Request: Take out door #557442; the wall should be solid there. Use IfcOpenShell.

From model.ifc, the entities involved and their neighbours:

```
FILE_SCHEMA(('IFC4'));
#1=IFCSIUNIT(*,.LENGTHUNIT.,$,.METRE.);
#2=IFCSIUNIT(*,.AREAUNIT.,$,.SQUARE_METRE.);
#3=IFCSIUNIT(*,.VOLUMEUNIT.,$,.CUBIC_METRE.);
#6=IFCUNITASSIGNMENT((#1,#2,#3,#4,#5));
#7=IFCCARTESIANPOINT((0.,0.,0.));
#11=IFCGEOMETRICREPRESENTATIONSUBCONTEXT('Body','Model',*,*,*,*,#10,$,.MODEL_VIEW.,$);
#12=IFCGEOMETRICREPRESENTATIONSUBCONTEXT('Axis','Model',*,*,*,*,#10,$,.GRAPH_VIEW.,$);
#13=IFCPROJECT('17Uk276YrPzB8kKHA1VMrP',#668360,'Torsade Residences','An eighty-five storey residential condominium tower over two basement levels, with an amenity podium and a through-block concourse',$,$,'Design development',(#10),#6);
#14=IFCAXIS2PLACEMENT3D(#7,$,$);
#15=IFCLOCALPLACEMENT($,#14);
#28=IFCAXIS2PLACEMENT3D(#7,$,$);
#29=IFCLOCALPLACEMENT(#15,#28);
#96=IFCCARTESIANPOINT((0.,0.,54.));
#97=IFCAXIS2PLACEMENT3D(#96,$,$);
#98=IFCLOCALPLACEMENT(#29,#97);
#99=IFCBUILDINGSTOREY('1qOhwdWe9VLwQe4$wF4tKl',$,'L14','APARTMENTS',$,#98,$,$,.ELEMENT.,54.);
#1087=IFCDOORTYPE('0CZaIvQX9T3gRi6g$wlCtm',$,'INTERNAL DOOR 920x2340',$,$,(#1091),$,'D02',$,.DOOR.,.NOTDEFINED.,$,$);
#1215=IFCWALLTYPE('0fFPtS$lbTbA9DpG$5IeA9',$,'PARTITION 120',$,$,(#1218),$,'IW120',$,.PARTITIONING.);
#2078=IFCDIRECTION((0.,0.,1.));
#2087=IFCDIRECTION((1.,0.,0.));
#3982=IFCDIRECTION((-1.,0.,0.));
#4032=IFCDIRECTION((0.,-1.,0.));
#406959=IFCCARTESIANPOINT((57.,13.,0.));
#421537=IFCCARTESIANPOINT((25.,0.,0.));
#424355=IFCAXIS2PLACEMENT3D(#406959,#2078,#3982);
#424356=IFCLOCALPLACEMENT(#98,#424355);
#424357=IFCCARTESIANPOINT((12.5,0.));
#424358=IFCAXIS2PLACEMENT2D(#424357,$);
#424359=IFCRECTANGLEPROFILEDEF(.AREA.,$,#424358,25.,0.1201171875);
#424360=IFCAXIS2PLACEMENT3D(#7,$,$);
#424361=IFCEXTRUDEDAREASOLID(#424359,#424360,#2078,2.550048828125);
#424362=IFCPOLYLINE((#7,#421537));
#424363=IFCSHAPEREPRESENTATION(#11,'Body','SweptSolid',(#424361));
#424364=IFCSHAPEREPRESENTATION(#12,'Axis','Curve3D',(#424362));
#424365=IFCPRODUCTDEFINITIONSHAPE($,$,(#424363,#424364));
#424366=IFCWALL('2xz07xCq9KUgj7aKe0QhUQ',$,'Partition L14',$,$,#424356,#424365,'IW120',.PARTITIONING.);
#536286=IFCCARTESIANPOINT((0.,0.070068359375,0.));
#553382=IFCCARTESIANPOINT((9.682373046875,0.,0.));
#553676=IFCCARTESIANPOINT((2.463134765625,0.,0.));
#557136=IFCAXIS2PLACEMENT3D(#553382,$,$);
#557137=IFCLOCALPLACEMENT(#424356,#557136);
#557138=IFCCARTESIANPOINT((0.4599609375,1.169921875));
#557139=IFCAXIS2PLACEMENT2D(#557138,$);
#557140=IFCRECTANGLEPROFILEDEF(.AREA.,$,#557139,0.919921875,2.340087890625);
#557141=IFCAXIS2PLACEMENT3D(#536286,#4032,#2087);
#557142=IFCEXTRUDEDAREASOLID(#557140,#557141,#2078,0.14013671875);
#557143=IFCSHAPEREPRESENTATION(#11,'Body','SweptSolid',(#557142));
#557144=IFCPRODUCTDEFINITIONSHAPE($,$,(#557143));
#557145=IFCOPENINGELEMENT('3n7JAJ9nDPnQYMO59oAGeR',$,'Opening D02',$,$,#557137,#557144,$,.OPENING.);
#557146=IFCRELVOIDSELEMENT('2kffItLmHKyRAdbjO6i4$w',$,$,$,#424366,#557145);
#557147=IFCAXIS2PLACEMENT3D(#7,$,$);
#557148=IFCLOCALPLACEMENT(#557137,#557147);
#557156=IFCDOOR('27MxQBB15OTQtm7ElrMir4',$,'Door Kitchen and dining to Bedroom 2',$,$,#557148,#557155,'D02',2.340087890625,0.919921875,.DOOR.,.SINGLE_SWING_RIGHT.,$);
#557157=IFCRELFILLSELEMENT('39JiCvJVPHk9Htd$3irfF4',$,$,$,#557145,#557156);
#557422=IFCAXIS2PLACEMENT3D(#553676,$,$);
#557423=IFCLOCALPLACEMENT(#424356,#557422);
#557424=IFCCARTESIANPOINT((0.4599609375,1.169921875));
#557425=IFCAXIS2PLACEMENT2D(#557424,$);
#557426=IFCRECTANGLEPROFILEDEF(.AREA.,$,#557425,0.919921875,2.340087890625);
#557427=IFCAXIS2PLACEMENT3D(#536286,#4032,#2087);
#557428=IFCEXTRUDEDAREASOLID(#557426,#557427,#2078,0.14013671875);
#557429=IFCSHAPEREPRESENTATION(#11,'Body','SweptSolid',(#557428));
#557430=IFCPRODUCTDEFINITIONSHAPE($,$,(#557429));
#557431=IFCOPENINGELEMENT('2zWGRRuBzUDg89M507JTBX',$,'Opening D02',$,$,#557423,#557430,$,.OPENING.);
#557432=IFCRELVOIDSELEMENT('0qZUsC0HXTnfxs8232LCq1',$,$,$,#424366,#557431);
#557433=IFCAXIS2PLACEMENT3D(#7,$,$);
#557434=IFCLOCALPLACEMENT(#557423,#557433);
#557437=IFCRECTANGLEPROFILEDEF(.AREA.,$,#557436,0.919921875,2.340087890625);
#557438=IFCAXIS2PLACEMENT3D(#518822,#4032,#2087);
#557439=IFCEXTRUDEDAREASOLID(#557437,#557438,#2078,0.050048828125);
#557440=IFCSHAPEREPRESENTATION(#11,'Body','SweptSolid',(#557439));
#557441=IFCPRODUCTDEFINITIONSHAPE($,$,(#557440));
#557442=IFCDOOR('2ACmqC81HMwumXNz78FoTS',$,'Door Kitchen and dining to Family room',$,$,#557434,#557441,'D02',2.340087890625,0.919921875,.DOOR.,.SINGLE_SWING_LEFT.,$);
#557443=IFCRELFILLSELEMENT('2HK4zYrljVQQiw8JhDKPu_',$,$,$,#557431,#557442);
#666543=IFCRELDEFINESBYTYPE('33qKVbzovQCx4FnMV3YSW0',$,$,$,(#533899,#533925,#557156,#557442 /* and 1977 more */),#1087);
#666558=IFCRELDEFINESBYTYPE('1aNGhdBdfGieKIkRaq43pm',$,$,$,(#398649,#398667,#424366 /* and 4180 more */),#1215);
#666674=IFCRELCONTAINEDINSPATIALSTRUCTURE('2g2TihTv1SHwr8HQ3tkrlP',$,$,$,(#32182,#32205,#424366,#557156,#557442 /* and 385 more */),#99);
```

```python
import ifcopenshell
import ifcopenshell.api.feature
import ifcopenshell.api.root
import ifcopenshell.geom
import ifcopenshell.util.shape

model = ifcopenshell.open("model.ifc")
settings = ifcopenshell.geom.settings()


def volume(element):
    """Net volume in cubic metres, openings subtracted."""
    shape = ifcopenshell.geom.create_shape(settings, element)
    return ifcopenshell.util.shape.get_volume(shape.geometry)


door = model.by_id(557442)
opening = door.FillsVoids[0].RelatingOpeningElement
wall = opening.VoidsElements[0].RelatingBuildingElement
before = volume(wall)

ifcopenshell.api.root.remove_product(model, product=door)
ifcopenshell.api.feature.remove_feature(model, feature=opening)

after = volume(wall)

print(f"wall volume {before:.3f} -> {after:.3f} m3")

model.write("model_rev.ifc")
```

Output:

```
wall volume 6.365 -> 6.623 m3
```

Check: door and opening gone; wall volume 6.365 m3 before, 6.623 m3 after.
